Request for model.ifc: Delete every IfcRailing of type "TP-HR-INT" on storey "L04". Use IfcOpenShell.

First a look at what the model holds.

```python
import ifcopenshell
import ifcopenshell.util.element

model = ifcopenshell.open("model.ifc")
print(model.schema)
storey = next(s for s in model.by_type("IfcBuildingStorey") if s.Name == "L04")
railings = [e for e in ifcopenshell.util.element.get_decomposition(storey) if e.is_a("IfcRailing")]
seen = {}
for e in railings:
    element_type = ifcopenshell.util.element.get_type(e)
    name = element_type.Name if element_type not in (None, e) else None
    seen[name] = seen.get(name, 0) + 1
for name, count in sorted(seen.items(), key=str):
    print(count, "x", name)
```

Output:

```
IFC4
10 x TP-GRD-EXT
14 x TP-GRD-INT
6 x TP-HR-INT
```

```python
import ifcopenshell
import ifcopenshell.api.root
import ifcopenshell.util.element

model = ifcopenshell.open("model.ifc")

storey = next(s for s in model.by_type("IfcBuildingStorey") if s.Name == "L04")
railings = [e for e in ifcopenshell.util.element.get_decomposition(storey) if e.is_a("IfcRailing")]
targets = [e for e in railings if (t := ifcopenshell.util.element.get_type(e)) not in (None, e) and t.Name == "TP-HR-INT"]

for e in targets:
    ifcopenshell.api.root.remove_product(model, product=e)
print(len(targets), "removed")

model.write("model_updated.ifc")
```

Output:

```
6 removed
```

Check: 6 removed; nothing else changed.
